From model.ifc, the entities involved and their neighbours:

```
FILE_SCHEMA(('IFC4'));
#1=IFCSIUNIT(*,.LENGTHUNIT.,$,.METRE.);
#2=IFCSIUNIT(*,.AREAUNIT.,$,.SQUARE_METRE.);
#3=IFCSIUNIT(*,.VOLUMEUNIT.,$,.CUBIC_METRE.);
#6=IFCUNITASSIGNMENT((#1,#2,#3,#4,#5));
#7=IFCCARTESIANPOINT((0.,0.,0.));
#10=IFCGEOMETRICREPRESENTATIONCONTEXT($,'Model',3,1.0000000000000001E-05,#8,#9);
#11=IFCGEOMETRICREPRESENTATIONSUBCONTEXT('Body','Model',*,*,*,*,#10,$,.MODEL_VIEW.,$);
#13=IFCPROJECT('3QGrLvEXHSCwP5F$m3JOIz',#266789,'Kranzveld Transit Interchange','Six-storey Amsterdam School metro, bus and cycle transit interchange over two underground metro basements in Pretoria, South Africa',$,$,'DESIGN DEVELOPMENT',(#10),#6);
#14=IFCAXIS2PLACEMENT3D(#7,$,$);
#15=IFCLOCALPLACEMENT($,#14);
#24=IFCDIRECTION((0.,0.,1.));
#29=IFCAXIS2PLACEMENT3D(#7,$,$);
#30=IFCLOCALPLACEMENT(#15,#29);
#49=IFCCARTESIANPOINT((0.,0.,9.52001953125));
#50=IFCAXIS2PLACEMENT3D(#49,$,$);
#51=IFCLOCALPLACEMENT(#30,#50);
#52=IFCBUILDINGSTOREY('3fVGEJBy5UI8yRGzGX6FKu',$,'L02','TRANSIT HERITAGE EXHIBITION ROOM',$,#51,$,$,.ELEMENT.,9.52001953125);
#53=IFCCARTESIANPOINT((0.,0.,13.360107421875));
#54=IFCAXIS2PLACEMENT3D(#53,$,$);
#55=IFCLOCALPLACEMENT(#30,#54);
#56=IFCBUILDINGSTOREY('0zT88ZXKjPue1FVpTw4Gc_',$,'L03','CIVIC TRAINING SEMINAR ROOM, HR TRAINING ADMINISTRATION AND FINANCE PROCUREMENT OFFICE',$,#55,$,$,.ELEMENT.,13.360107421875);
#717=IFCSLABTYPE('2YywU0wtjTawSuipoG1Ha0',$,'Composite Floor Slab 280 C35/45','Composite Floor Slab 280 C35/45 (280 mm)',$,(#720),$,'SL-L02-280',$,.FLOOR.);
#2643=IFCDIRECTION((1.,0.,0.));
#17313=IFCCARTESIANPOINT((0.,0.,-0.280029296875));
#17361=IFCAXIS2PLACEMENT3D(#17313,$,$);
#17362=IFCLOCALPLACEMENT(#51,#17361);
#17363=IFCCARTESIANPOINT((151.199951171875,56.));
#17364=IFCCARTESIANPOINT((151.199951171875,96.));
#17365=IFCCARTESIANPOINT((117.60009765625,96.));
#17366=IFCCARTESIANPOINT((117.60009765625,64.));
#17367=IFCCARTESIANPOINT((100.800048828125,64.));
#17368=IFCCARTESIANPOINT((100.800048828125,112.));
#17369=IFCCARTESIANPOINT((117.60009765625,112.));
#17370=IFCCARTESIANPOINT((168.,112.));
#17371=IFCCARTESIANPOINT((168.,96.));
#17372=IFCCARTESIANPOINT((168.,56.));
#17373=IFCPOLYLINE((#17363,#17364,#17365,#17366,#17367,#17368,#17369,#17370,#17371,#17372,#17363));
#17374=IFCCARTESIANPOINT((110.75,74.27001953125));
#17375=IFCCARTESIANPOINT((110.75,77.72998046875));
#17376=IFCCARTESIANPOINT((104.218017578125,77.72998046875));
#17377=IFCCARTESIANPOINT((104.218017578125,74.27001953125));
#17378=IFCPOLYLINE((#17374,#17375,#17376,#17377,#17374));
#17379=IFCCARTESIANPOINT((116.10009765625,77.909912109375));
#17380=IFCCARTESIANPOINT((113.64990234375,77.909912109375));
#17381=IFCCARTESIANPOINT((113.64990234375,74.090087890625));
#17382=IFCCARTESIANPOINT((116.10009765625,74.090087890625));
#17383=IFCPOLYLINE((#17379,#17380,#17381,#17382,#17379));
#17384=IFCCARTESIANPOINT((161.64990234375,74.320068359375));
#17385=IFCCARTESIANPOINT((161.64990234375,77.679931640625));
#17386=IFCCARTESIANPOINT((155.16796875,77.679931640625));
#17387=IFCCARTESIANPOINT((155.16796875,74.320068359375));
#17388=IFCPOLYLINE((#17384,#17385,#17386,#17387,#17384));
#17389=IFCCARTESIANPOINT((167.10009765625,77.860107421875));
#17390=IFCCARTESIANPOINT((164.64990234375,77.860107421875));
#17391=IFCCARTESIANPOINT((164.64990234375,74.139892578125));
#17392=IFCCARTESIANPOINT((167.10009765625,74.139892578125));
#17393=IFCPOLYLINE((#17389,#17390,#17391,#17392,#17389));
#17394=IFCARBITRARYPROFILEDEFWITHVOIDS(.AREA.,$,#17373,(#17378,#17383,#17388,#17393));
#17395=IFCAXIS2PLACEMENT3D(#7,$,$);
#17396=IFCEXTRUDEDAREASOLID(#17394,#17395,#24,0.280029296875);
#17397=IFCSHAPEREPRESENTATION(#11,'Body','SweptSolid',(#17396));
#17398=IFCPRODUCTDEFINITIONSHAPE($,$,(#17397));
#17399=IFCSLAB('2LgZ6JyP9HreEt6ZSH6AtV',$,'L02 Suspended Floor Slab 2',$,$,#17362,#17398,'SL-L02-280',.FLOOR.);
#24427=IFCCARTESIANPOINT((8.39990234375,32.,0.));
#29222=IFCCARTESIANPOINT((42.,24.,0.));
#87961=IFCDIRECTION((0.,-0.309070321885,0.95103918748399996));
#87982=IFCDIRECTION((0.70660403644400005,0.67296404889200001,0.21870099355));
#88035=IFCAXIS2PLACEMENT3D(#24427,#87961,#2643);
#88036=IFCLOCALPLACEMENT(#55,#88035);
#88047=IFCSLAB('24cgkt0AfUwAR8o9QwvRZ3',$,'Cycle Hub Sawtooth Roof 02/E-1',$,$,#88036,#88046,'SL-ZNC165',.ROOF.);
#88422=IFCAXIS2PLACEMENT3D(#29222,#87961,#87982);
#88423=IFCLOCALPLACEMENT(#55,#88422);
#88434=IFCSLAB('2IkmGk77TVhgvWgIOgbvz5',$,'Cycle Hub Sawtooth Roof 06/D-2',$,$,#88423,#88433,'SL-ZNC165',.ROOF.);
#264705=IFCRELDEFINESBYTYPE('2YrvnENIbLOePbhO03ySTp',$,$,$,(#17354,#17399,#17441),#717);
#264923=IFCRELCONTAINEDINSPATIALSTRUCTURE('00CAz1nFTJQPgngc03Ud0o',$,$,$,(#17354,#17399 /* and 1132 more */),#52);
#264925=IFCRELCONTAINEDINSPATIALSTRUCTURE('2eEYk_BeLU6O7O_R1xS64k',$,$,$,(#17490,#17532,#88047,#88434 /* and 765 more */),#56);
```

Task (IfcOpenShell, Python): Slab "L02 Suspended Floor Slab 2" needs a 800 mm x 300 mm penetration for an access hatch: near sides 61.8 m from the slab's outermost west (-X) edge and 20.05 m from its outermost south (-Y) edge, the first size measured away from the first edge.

```python
import numpy as np
import ifcopenshell
import ifcopenshell.api.feature
import ifcopenshell.api.geometry
import ifcopenshell.api.root
import ifcopenshell.geom
import ifcopenshell.util.placement
import ifcopenshell.util.representation
import ifcopenshell.util.shape
import ifcopenshell.util.unit

model = ifcopenshell.open("model.ifc")
unit_scale = ifcopenshell.util.unit.calculate_unit_scale(model)
settings = ifcopenshell.geom.settings()


def volume(element):
    """Net volume in cubic metres, openings subtracted."""
    shape = ifcopenshell.geom.create_shape(settings, element)
    return ifcopenshell.util.shape.get_volume(shape.geometry)


slab = model.by_guid("2LgZ6JyP9HreEt6ZSH6AtV")
before = volume(slab)

# Extent in the slab's own axes, in metres. The edges named are its -X and -Y sides.
slab_shape = ifcopenshell.geom.create_shape(settings, slab)
vertices = ifcopenshell.util.shape.get_vertices(slab_shape.geometry)
x_min, y_min, bottom = vertices.min(axis=0)
top = vertices[:, 2].max()

opening = ifcopenshell.api.root.create_entity(model, ifc_class="IfcOpeningElement", name="Access hatch opening", predefined_type="OPENING")
context = ifcopenshell.util.representation.get_context(model, "Model", "Body", "MODEL_VIEW")
width, depth = 0.8, 0.3
outline = [(0.0, 0.0), (width, 0.0), (width, depth), (0.0, depth), (0.0, 0.0)]
# Overshoot both faces by 50 mm so the cut is clean.
shape = ifcopenshell.api.geometry.add_slab_representation(
    model, context=context, depth=top - bottom + 0.1, polyline=outline
)
ifcopenshell.api.geometry.assign_representation(model, product=opening, representation=shape)

matrix = ifcopenshell.util.placement.get_local_placement(slab.ObjectPlacement)
matrix[:, 3] = matrix @ np.append(np.array([x_min + 61.8, y_min + 20.05, bottom - 0.05]) / unit_scale, 1.0)
ifcopenshell.api.geometry.edit_object_placement(model, product=opening, matrix=matrix, is_si=False)
ifcopenshell.api.feature.add_feature(model, feature=opening, element=slab)

after = volume(slab)

print(f"slab volume {before:.3f} -> {after:.3f} m3")

model.write("model_edited.ifc")
```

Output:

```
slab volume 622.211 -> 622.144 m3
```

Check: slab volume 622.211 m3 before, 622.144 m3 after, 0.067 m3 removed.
